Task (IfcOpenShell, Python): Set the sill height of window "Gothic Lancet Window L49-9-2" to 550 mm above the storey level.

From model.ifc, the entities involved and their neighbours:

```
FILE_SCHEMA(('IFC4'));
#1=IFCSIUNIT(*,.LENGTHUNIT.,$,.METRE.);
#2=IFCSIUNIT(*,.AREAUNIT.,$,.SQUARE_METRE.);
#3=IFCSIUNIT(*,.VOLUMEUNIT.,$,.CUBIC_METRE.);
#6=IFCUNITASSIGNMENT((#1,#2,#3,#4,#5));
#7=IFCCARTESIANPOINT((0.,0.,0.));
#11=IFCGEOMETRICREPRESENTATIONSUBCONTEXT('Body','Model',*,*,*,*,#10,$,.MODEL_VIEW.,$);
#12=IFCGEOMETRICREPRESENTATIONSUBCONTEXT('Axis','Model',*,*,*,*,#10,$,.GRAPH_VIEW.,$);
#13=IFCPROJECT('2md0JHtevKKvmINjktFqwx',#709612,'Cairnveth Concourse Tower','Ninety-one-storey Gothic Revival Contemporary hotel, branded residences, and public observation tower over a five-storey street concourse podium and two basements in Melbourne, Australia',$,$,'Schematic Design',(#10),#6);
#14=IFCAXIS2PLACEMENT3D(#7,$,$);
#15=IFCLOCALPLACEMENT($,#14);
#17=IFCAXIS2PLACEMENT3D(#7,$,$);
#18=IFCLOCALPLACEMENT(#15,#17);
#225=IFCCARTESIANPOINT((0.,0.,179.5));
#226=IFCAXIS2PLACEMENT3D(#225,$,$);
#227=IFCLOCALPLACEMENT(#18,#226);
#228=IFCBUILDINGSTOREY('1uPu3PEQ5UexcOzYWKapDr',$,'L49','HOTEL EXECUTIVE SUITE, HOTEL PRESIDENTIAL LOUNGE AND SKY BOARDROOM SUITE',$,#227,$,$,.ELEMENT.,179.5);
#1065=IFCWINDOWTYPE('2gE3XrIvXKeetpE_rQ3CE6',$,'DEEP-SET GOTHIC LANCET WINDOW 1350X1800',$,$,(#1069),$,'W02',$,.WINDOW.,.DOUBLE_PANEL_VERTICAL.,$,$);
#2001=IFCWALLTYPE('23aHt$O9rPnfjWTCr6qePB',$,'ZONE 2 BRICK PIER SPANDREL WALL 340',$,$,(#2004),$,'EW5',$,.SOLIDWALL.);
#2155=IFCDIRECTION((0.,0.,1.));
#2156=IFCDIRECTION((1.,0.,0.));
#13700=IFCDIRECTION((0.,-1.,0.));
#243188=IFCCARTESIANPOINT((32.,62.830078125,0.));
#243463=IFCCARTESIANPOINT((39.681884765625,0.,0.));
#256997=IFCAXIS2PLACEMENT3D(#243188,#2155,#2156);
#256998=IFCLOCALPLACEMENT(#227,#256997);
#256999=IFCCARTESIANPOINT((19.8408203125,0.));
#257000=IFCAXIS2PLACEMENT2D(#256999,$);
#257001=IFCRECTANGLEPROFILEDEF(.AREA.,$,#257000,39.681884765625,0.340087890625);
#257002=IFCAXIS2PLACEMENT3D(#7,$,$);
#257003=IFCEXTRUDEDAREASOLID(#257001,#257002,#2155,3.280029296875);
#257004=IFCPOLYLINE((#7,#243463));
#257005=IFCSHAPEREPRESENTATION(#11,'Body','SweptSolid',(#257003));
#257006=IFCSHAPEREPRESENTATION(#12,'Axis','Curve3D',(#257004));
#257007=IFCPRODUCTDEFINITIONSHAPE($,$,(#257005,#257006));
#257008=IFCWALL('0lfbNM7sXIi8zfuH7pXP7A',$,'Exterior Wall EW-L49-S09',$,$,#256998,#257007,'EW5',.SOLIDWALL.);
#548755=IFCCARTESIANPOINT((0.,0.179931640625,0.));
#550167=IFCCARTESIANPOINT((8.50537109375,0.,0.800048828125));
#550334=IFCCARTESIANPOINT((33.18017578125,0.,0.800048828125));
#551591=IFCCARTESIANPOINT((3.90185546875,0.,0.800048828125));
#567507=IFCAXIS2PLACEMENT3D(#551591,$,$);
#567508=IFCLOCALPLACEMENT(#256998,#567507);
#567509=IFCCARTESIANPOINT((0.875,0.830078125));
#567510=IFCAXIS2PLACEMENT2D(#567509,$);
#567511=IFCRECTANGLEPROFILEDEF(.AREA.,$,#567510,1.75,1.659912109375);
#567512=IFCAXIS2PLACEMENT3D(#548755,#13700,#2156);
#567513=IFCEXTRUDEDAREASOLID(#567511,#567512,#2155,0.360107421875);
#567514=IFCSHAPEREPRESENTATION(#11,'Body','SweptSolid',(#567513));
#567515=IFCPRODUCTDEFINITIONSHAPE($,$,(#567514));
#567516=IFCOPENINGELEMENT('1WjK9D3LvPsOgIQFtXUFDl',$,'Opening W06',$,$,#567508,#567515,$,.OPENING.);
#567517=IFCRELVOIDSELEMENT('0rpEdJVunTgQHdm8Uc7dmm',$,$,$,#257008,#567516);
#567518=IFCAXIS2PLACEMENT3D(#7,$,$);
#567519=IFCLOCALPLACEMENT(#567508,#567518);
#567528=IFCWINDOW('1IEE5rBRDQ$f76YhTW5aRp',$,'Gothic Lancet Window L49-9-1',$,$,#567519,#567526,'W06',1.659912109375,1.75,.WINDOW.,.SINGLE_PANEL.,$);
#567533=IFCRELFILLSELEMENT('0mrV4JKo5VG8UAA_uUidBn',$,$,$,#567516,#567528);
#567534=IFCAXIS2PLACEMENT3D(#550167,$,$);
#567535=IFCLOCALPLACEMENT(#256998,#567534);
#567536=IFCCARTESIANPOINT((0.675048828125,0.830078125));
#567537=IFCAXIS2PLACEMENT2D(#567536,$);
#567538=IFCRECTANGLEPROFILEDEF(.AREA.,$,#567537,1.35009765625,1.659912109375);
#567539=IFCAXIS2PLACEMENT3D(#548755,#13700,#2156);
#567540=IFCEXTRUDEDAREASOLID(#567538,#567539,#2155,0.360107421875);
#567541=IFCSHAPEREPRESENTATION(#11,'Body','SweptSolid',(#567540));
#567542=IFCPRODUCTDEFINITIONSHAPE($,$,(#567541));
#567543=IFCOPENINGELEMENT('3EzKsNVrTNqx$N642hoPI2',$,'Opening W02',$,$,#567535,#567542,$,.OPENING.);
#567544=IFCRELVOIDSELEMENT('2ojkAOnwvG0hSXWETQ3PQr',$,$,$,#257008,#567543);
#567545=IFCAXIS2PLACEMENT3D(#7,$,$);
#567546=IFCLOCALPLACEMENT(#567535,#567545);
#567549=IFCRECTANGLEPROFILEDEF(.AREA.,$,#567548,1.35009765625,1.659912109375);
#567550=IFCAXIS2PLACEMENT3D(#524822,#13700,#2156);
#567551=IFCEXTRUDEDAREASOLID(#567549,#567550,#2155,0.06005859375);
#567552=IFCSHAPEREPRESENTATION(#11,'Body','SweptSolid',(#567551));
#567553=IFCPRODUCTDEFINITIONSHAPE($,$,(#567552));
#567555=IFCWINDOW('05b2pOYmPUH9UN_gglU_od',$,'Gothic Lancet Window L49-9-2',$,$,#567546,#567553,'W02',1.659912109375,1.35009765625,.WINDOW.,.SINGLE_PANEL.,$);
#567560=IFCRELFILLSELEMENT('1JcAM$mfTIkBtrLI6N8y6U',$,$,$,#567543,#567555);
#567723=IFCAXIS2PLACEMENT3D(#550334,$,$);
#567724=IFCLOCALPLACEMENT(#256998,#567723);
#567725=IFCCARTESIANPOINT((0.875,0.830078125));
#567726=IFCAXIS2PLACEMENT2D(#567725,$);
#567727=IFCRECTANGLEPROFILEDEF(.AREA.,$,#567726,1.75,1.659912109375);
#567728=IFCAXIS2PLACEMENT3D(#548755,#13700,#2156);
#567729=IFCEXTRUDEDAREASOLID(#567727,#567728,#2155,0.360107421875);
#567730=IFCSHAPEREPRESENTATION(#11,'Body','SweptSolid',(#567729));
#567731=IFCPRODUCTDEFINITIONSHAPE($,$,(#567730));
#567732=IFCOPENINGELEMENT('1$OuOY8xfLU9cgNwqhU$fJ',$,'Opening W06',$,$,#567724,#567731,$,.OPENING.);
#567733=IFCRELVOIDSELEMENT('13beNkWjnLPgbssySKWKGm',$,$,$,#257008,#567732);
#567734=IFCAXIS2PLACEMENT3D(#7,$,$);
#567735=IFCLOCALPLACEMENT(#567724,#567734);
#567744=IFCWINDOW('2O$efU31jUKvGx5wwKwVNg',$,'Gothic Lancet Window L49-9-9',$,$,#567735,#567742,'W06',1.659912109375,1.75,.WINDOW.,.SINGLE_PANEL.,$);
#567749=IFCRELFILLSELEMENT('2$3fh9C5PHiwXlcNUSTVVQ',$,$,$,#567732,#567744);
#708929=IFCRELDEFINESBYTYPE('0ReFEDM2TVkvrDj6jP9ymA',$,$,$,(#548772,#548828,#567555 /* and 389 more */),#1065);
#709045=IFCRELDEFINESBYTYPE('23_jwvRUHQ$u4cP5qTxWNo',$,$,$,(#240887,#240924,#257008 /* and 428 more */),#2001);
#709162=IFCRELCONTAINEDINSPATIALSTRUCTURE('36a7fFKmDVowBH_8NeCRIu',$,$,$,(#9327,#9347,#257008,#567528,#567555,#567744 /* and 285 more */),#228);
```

```python
import numpy as np
import ifcopenshell
import ifcopenshell.api.geometry
import ifcopenshell.geom
import ifcopenshell.util.element
import ifcopenshell.util.placement
import ifcopenshell.util.shape
import ifcopenshell.util.unit

model = ifcopenshell.open("model.ifc")
unit_scale = ifcopenshell.util.unit.calculate_unit_scale(model)

window = model.by_id(567555)
opening = window.FillsVoids[0].RelatingOpeningElement
storey = ifcopenshell.util.element.get_container(window, ifc_class="IfcBuildingStorey")
level = ifcopenshell.util.placement.get_local_placement(storey.ObjectPlacement)[2, 3]

# The opening's origin need not be at the sill, so measure its lowest point.
shape = ifcopenshell.geom.create_shape(ifcopenshell.geom.settings(), opening)
bottom = ifcopenshell.util.shape.get_shape_bottom_elevation(shape, shape.geometry) / unit_scale
dz = level + 0.55 - bottom

shift = np.array([0.0, 0.0, dz])
# The window is placed relative to its opening, so it follows when the opening moves.
matrix = ifcopenshell.util.placement.get_local_placement(opening.ObjectPlacement)
matrix[:3, 3] += shift
ifcopenshell.api.geometry.edit_object_placement(
    model, product=opening, matrix=matrix, is_si=False, should_transform_children=True
)

print(f"moved by {dz * unit_scale:+.3f} m")

model.write("model_v2.ifc")
```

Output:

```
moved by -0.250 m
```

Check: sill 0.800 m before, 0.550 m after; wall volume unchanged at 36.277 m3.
